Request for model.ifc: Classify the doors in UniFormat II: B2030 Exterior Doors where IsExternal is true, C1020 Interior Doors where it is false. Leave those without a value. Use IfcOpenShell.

First a look at what the model holds.

```python
import ifcopenshell
import ifcopenshell.util.element

model = ifcopenshell.open("model.ifc")
print(model.schema)
print("classifications:", [c.Name for c in model.by_type("IfcClassification")])
values = [ifcopenshell.util.element.get_pset(e, "Pset_DoorCommon", "IsExternal") for e in model.by_type("IfcDoor")]
for value in (True, False, None):
    print("IsExternal", value, values.count(value))
```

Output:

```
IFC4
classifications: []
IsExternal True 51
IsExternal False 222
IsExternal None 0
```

```python
import ifcopenshell
import ifcopenshell.api.classification
import ifcopenshell.util.element

model = ifcopenshell.open("model.ifc")

system = ifcopenshell.api.classification.add_classification(model, classification="UniFormat II")

doors = model.by_type("IfcDoor")
external = {e: ifcopenshell.util.element.get_pset(e, "Pset_DoorCommon", "IsExternal") for e in doors}
for flag, code, name in ((True, "B2030", "Exterior Doors"), (False, "C1020", "Interior Doors")):
    products = [e for e in doors if external[e] is flag]
    ifcopenshell.api.classification.add_reference(
        model, products=products, classification=system, identification=code, name=name
    )
    print(code, len(products))

model.write("model_updated.ifc")
```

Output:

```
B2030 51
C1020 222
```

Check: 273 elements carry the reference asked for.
